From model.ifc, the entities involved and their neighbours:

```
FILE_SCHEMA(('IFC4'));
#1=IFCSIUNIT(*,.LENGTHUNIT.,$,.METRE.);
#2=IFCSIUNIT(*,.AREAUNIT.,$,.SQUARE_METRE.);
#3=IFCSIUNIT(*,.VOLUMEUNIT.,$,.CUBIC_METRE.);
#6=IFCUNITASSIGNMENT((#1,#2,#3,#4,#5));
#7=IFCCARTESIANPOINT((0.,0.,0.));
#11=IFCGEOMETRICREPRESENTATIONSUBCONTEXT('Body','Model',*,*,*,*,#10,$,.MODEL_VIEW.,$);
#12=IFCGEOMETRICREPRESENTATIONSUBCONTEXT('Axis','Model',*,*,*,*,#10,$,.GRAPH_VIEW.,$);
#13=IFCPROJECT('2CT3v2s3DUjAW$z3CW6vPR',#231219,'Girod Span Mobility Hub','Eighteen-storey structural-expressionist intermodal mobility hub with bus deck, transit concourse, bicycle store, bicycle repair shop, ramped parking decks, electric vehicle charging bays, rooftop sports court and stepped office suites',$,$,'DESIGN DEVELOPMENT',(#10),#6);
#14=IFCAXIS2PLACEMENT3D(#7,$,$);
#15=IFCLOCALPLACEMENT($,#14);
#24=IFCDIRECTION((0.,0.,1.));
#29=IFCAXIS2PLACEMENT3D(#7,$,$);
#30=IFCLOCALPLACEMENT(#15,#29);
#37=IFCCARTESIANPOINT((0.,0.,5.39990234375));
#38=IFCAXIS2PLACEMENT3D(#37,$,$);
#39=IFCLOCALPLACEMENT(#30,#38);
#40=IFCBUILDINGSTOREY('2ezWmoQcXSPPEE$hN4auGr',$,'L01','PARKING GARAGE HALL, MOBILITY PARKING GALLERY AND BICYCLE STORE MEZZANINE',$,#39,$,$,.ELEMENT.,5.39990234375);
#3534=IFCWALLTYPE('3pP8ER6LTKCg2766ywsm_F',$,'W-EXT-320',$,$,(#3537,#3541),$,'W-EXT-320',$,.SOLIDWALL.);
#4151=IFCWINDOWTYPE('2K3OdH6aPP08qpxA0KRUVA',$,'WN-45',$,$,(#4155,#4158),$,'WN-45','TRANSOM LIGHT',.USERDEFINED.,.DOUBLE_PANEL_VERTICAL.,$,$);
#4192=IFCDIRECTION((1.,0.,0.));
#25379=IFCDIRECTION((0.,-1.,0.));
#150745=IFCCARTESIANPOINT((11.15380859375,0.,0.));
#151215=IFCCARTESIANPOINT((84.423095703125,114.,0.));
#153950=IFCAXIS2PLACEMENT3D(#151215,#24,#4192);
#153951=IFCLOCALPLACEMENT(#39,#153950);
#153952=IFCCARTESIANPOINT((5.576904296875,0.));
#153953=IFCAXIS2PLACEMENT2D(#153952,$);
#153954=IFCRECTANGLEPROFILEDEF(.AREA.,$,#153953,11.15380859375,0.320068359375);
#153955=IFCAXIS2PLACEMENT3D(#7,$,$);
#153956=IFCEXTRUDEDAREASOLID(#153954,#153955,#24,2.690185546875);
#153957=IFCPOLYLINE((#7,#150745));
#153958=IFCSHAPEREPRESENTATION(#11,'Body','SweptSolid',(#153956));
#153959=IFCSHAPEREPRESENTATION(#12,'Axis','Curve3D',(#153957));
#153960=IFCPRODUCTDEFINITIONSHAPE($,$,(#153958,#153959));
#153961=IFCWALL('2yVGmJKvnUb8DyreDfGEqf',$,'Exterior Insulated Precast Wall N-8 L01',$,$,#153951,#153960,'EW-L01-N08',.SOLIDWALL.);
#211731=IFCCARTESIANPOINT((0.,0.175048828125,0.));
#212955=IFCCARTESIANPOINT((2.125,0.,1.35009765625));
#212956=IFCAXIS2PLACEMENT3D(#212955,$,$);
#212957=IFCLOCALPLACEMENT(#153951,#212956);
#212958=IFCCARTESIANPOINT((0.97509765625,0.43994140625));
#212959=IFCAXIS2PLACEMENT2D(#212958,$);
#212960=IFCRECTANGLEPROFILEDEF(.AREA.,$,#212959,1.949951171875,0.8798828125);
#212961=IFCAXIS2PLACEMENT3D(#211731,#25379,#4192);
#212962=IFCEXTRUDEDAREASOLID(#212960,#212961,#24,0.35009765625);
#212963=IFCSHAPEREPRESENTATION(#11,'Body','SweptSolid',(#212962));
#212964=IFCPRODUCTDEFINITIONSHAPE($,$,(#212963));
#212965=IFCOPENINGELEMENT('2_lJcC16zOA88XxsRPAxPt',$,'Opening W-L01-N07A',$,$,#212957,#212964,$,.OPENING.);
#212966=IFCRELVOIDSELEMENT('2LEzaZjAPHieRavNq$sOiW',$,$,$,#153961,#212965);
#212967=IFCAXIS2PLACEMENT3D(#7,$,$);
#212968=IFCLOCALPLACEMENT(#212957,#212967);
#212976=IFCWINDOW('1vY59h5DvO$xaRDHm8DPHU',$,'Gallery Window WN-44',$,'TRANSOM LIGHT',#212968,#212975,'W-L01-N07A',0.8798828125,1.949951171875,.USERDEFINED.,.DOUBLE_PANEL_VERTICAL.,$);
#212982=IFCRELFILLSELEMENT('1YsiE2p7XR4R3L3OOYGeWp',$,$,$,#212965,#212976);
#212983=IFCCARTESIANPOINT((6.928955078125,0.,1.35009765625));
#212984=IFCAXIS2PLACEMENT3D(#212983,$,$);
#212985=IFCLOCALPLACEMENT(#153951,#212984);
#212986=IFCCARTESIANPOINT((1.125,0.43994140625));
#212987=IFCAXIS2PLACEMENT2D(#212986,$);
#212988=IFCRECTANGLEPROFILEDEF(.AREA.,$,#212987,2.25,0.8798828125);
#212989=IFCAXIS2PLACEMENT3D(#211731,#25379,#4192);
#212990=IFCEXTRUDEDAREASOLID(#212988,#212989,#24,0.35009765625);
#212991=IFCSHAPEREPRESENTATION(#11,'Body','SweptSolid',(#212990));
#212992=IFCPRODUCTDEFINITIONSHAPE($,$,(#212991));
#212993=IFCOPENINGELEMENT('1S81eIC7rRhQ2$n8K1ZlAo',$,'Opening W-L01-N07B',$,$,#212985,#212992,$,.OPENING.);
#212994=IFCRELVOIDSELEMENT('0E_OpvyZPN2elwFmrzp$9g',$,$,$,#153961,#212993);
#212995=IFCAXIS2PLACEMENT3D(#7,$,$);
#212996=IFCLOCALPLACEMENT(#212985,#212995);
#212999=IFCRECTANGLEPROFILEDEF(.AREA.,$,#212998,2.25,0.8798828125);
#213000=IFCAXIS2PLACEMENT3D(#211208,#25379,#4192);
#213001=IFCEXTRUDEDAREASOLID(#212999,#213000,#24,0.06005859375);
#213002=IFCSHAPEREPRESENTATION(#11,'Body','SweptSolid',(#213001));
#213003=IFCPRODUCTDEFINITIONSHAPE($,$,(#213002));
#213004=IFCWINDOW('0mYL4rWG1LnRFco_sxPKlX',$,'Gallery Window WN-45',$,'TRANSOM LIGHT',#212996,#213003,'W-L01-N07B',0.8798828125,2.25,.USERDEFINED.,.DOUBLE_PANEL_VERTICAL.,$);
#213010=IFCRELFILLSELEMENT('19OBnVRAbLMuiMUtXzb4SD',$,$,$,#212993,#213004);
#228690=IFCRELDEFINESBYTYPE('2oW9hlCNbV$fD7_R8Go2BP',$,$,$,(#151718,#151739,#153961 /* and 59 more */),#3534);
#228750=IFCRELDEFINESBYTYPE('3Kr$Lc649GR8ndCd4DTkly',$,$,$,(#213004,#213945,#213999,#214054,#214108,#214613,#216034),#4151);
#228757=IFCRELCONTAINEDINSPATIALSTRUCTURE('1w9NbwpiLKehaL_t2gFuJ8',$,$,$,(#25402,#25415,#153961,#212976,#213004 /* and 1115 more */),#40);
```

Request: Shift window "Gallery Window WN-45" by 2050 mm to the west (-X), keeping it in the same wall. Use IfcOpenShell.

```python
import ifcopenshell
import ifcopenshell.api.geometry
import ifcopenshell.util.placement
import ifcopenshell.util.unit

model = ifcopenshell.open("model.ifc")
unit_scale = ifcopenshell.util.unit.calculate_unit_scale(model)

window = model.by_id(213004)
opening = window.FillsVoids[0].RelatingOpeningElement
wall = opening.VoidsElements[0].RelatingBuildingElement

wall_matrix = ifcopenshell.util.placement.get_local_placement(wall.ObjectPlacement)
shift = wall_matrix[:3, 0] * -2.05 / unit_scale
before = ifcopenshell.util.placement.get_local_placement(window.ObjectPlacement)[:3, 3].copy()

# The window is placed relative to its opening, so it follows when the opening moves.
matrix = ifcopenshell.util.placement.get_local_placement(opening.ObjectPlacement)
matrix[:3, 3] += shift
ifcopenshell.api.geometry.edit_object_placement(
    model, product=opening, matrix=matrix, is_si=False, should_transform_children=True
)

after = ifcopenshell.util.placement.get_local_placement(window.ObjectPlacement)[:3, 3]
print("window moved by", (after - before).round(3) + 0.0)

model.write("model_rev.ifc")
```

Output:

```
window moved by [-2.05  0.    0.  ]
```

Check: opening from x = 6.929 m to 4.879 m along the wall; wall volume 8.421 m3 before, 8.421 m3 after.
